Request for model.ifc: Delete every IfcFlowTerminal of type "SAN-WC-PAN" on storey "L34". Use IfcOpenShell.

First a look at what the model holds.

```python
import ifcopenshell
import ifcopenshell.util.element

model = ifcopenshell.open("model.ifc")
print(model.schema)
storey = next(s for s in model.by_type("IfcBuildingStorey") if s.Name == "L34")
terminals = [e for e in ifcopenshell.util.element.get_decomposition(storey) if e.is_a("IfcFlowTerminal")]
seen = {}
for e in terminals:
    element_type = ifcopenshell.util.element.get_type(e)
    name = element_type.Name if element_type not in (None, e) else None
    seen[name] = seen.get(name, 0) + 1
for name, count in sorted(seen.items(), key=str):
    print(count, "x", name)
```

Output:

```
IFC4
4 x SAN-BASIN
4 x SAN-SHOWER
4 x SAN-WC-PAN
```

```python
import ifcopenshell
import ifcopenshell.api.root
import ifcopenshell.util.element

model = ifcopenshell.open("model.ifc")

storey = next(s for s in model.by_type("IfcBuildingStorey") if s.Name == "L34")
terminals = [e for e in ifcopenshell.util.element.get_decomposition(storey) if e.is_a("IfcFlowTerminal")]
targets = [e for e in terminals if (t := ifcopenshell.util.element.get_type(e)) not in (None, e) and t.Name == "SAN-WC-PAN"]

for e in targets:
    ifcopenshell.api.root.remove_product(model, product=e)
print(len(targets), "removed")

model.write("model_rev.ifc")
```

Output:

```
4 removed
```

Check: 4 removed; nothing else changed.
